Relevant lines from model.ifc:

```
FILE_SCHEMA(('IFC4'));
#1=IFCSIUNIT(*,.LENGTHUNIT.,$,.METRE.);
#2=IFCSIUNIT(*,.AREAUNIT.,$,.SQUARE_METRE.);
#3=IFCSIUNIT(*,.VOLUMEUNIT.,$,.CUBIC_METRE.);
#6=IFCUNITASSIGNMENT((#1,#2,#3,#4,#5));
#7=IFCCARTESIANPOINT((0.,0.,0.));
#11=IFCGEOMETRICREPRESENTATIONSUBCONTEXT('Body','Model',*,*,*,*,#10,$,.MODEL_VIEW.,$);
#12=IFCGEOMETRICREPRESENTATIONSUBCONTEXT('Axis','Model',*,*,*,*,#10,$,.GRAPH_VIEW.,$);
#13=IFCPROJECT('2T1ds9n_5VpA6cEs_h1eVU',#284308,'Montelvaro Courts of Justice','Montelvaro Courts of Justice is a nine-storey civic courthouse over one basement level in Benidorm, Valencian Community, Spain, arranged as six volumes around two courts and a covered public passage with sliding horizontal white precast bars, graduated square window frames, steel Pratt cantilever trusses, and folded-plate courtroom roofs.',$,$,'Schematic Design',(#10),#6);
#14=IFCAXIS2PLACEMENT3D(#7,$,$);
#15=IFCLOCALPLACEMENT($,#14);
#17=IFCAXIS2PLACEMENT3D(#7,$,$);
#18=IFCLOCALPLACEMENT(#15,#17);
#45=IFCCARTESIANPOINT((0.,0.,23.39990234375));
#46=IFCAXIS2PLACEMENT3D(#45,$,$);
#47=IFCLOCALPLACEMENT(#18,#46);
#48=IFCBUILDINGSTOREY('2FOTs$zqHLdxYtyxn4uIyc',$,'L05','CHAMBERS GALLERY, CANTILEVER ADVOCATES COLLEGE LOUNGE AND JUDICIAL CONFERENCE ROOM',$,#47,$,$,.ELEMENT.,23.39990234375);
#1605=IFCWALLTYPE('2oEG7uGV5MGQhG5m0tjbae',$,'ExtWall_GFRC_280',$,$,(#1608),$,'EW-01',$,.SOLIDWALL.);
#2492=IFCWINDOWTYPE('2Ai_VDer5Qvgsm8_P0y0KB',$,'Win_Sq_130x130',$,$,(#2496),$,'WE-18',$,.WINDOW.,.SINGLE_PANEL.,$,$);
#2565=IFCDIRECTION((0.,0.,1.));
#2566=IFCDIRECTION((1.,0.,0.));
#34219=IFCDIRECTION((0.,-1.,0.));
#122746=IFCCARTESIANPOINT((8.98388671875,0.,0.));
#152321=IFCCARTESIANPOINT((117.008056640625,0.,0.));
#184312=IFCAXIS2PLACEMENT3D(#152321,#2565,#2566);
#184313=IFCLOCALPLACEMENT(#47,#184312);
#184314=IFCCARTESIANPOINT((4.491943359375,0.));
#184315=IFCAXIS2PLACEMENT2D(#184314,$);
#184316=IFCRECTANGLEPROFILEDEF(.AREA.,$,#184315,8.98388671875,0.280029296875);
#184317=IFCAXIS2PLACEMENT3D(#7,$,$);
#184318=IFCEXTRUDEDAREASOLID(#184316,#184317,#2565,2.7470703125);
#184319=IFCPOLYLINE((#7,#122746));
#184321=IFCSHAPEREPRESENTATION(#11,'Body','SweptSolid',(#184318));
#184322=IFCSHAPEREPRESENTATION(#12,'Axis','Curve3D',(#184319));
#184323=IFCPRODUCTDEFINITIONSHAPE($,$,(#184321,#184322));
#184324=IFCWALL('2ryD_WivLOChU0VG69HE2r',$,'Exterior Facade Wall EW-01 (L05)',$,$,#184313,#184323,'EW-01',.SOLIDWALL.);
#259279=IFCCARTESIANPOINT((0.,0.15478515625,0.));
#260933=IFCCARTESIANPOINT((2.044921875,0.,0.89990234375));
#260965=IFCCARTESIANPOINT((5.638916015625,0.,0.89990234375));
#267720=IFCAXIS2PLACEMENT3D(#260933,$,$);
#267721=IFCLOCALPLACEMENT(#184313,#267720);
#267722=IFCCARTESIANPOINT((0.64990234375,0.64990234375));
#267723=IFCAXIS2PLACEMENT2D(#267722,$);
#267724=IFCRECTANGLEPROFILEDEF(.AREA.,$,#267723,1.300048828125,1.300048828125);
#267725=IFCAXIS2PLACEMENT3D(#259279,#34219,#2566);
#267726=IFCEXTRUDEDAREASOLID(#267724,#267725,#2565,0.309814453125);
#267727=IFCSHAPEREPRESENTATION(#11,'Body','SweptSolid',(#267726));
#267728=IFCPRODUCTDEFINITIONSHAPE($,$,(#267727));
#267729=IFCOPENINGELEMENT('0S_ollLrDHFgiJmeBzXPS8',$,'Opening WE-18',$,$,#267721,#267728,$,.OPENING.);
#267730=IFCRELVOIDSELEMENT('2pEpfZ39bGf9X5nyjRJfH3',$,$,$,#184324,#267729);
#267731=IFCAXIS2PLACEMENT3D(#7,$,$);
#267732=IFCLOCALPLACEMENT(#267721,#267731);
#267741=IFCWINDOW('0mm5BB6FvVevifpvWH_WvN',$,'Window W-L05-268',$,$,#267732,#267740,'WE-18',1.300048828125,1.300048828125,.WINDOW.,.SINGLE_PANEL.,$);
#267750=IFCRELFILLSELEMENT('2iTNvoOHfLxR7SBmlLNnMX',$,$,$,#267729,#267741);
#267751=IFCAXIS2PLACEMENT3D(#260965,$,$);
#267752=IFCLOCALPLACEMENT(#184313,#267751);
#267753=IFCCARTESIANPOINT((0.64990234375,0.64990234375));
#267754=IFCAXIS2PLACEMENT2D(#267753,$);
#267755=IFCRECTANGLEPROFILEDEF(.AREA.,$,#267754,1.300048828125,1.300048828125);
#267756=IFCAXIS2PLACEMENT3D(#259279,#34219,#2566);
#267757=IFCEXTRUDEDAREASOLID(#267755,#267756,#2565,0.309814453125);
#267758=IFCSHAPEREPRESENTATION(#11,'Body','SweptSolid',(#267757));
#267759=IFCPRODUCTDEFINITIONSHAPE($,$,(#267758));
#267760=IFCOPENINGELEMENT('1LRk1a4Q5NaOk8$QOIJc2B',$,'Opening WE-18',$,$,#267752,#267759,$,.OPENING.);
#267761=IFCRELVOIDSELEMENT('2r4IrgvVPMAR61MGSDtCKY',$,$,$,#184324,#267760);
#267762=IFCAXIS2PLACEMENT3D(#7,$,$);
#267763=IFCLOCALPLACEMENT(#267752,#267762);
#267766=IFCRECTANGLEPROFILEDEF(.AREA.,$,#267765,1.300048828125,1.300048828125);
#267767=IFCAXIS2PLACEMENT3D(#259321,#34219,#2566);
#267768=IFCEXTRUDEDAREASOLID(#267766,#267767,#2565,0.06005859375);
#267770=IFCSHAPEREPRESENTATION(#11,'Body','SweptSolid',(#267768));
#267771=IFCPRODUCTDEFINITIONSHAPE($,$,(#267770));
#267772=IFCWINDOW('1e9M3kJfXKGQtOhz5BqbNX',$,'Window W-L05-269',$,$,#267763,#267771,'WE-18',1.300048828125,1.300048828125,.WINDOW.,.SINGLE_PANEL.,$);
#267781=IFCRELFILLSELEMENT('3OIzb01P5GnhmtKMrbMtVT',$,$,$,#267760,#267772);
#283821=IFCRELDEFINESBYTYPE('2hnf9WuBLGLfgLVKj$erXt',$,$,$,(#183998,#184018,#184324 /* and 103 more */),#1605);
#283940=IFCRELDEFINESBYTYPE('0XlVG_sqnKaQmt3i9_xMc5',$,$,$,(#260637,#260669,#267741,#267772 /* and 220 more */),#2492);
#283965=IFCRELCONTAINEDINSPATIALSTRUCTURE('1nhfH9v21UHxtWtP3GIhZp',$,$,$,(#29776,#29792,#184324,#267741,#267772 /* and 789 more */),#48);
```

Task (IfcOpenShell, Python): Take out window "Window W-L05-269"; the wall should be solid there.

```python
import ifcopenshell
import ifcopenshell.api.feature
import ifcopenshell.api.root
import ifcopenshell.geom
import ifcopenshell.util.shape

model = ifcopenshell.open("model.ifc")
settings = ifcopenshell.geom.settings()


def volume(element):
    """Net volume in cubic metres, openings subtracted."""
    shape = ifcopenshell.geom.create_shape(settings, element)
    return ifcopenshell.util.shape.get_volume(shape.geometry)


window = model.by_guid("1e9M3kJfXKGQtOhz5BqbNX")
opening = window.FillsVoids[0].RelatingOpeningElement
wall = opening.VoidsElements[0].RelatingBuildingElement
before = volume(wall)

ifcopenshell.api.root.remove_product(model, product=window)
ifcopenshell.api.feature.remove_feature(model, feature=opening)

after = volume(wall)

print(f"wall volume {before:.3f} -> {after:.3f} m3")

model.write("model-out.ifc")
```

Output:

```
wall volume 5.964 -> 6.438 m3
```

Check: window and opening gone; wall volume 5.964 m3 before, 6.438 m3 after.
